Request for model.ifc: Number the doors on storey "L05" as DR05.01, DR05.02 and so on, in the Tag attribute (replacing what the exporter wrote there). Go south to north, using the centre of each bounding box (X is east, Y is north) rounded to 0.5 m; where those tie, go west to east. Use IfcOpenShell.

First a look at what the model holds.

```python
import ifcopenshell
import ifcopenshell.util.element
import ifcopenshell.util.placement

model = ifcopenshell.open("model.ifc")
print(model.schema)
storey = next(s for s in model.by_type("IfcBuildingStorey") if s.Name == "L05")
doors = [e for e in ifcopenshell.util.element.get_decomposition(storey) if e.is_a("IfcDoor")]
for e in sorted(doors, key=lambda e: e.id()):
    origin = ifcopenshell.util.placement.get_local_placement(e.ObjectPlacement)[:3, 3]
    print(e.id(), e.Tag, e.Name, origin.round(2) + 0.0, sep=" | ")
```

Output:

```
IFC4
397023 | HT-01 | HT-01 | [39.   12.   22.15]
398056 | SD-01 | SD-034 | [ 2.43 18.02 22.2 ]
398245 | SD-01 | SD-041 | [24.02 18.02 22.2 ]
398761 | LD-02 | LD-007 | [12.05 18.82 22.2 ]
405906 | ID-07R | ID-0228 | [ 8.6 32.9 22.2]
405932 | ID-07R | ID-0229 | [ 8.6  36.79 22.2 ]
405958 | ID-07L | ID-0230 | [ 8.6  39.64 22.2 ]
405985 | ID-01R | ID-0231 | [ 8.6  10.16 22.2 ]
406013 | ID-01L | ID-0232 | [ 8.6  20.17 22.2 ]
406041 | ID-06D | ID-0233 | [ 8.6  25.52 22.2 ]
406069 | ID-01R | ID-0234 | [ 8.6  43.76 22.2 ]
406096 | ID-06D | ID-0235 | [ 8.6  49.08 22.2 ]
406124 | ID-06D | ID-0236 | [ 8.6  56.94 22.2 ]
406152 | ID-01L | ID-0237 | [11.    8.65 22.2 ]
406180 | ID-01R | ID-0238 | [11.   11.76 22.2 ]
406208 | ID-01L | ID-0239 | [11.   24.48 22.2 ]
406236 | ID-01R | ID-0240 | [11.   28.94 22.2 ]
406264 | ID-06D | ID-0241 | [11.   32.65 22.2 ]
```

```python
import ifcopenshell
import ifcopenshell.geom
import ifcopenshell.util.element
import ifcopenshell.util.shape

model = ifcopenshell.open("model.ifc")
settings = ifcopenshell.geom.settings()
settings.set("use-world-coords", True)


def centre(element):
    shape = ifcopenshell.geom.create_shape(settings, element)
    return ifcopenshell.util.shape.get_bbox_centroid(shape.geometry)


storey = next(s for s in model.by_type("IfcBuildingStorey") if s.Name == "L05")
doors = [e for e in ifcopenshell.util.element.get_decomposition(storey) if e.is_a("IfcDoor")]

# Insertion points can sit at a corner or the storey origin, so sort by the geometry (in metres).
centres = {e: centre(e) for e in doors}
doors.sort(key=lambda e: (round(centres[e][1] / 0.5), centres[e][0]))

for i, e in enumerate(doors, start=1):
    number = f"DR05.{i:02d}"
    e.Tag = number
    print(e.id(), number)

model.write("model_v2.ifc")
```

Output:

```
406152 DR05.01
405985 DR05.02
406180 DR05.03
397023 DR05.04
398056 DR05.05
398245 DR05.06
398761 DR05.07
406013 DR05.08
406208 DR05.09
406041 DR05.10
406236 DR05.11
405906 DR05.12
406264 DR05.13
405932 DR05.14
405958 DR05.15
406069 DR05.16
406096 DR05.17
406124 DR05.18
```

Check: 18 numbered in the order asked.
